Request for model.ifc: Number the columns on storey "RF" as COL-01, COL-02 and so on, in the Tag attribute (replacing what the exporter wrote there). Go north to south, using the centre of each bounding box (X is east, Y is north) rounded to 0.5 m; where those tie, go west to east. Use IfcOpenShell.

First a look at what the model holds.

```python
import ifcopenshell
import ifcopenshell.util.element
import ifcopenshell.util.placement

model = ifcopenshell.open("model.ifc")
print(model.schema)
storey = next(s for s in model.by_type("IfcBuildingStorey") if s.Name == "RF")
columns = [e for e in ifcopenshell.util.element.get_decomposition(storey) if e.is_a("IfcColumn")]
for e in sorted(columns, key=lambda e: e.id()):
    origin = ifcopenshell.util.placement.get_local_placement(e.ObjectPlacement)[:3, 3]
    print(e.id(), e.Tag, e.Name, origin.round(2) + 0.0, sep=" | ")
```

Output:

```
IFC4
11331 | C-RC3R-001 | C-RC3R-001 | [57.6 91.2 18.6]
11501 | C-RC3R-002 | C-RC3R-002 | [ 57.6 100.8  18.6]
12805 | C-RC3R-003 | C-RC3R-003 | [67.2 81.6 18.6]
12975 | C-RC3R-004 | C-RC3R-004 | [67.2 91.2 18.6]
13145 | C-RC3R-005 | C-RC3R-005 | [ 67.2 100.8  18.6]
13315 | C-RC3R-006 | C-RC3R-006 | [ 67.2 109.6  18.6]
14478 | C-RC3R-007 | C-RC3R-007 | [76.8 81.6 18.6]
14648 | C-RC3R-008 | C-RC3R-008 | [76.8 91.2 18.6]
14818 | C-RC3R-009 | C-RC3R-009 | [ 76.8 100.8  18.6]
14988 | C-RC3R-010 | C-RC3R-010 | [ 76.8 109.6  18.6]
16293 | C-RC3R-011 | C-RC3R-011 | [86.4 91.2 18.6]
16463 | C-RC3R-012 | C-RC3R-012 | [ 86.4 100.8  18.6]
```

```python
import ifcopenshell
import ifcopenshell.geom
import ifcopenshell.util.element
import ifcopenshell.util.shape

model = ifcopenshell.open("model.ifc")
settings = ifcopenshell.geom.settings()
settings.set("use-world-coords", True)


def centre(element):
    shape = ifcopenshell.geom.create_shape(settings, element)
    return ifcopenshell.util.shape.get_bbox_centroid(shape.geometry)


storey = next(s for s in model.by_type("IfcBuildingStorey") if s.Name == "RF")
columns = [e for e in ifcopenshell.util.element.get_decomposition(storey) if e.is_a("IfcColumn")]

# Insertion points can sit at a corner or the storey origin, so sort by the geometry (in metres).
centres = {e: centre(e) for e in columns}
columns.sort(key=lambda e: (-round(centres[e][1] / 0.5), centres[e][0]))

for i, e in enumerate(columns, start=1):
    number = f"COL-{i:02d}"
    e.Tag = number
    print(e.id(), number)

model.write("model_v2.ifc")
```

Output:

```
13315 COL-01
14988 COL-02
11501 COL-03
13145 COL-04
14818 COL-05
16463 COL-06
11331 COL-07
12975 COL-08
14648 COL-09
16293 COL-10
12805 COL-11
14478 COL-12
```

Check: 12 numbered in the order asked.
